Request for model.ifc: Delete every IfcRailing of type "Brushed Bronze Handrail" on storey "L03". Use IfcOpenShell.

First a look at what the model holds.

```python
import ifcopenshell
import ifcopenshell.util.element

model = ifcopenshell.open("model.ifc")
print(model.schema)
storey = next(s for s in model.by_type("IfcBuildingStorey") if s.Name == "L03")
railings = [e for e in ifcopenshell.util.element.get_decomposition(storey) if e.is_a("IfcRailing")]
seen = {}
for e in railings:
    element_type = ifcopenshell.util.element.get_type(e)
    name = element_type.Name if element_type not in (None, e) else None
    seen[name] = seen.get(name, 0) + 1
for name, count in sorted(seen.items(), key=str):
    print(count, "x", name)
```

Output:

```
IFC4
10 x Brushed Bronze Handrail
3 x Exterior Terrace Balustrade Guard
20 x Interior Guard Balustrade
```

```python
import ifcopenshell
import ifcopenshell.api.root
import ifcopenshell.util.element

model = ifcopenshell.open("model.ifc")

storey = next(s for s in model.by_type("IfcBuildingStorey") if s.Name == "L03")
railings = [e for e in ifcopenshell.util.element.get_decomposition(storey) if e.is_a("IfcRailing")]
targets = [e for e in railings if (t := ifcopenshell.util.element.get_type(e)) not in (None, e) and t.Name == "Brushed Bronze Handrail"]

for e in targets:
    ifcopenshell.api.root.remove_product(model, product=e)
print(len(targets), "removed")

model.write("model_rev.ifc")
```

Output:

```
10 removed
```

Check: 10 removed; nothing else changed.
